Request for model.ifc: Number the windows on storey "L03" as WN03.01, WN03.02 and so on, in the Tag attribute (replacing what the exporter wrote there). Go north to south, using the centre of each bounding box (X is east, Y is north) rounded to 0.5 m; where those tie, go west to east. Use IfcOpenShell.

First a look at what the model holds.

```python
import ifcopenshell
import ifcopenshell.util.element
import ifcopenshell.util.placement

model = ifcopenshell.open("model.ifc")
print(model.schema)
storey = next(s for s in model.by_type("IfcBuildingStorey") if s.Name == "L03")
windows = [e for e in ifcopenshell.util.element.get_decomposition(storey) if e.is_a("IfcWindow")]
for e in sorted(windows, key=lambda e: e.id()):
    origin = ifcopenshell.util.placement.get_local_placement(e.ObjectPlacement)[:3, 3]
    print(e.id(), e.Tag, e.Name, origin.round(2) + 0.0, sep=" | ")
```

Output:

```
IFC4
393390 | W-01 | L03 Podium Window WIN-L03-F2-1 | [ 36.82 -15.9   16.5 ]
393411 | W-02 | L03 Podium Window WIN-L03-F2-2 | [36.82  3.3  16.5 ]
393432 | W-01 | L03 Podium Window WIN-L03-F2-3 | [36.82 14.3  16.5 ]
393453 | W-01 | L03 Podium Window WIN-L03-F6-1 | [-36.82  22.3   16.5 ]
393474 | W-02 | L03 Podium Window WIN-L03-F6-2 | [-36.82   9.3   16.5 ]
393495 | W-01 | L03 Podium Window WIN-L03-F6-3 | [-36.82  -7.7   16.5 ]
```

```python
import ifcopenshell
import ifcopenshell.geom
import ifcopenshell.util.element
import ifcopenshell.util.shape

model = ifcopenshell.open("model.ifc")
settings = ifcopenshell.geom.settings()
settings.set("use-world-coords", True)


def centre(element):
    shape = ifcopenshell.geom.create_shape(settings, element)
    return ifcopenshell.util.shape.get_bbox_centroid(shape.geometry)


storey = next(s for s in model.by_type("IfcBuildingStorey") if s.Name == "L03")
windows = [e for e in ifcopenshell.util.element.get_decomposition(storey) if e.is_a("IfcWindow")]

# Insertion points can sit at a corner or the storey origin, so sort by the geometry (in metres).
centres = {e: centre(e) for e in windows}
windows.sort(key=lambda e: (-round(centres[e][1] / 0.5), centres[e][0]))

for i, e in enumerate(windows, start=1):
    number = f"WN03.{i:02d}"
    e.Tag = number
    print(e.id(), number)

model.write("model-out.ifc")
```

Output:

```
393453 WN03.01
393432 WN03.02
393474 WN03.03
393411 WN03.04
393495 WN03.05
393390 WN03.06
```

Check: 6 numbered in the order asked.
